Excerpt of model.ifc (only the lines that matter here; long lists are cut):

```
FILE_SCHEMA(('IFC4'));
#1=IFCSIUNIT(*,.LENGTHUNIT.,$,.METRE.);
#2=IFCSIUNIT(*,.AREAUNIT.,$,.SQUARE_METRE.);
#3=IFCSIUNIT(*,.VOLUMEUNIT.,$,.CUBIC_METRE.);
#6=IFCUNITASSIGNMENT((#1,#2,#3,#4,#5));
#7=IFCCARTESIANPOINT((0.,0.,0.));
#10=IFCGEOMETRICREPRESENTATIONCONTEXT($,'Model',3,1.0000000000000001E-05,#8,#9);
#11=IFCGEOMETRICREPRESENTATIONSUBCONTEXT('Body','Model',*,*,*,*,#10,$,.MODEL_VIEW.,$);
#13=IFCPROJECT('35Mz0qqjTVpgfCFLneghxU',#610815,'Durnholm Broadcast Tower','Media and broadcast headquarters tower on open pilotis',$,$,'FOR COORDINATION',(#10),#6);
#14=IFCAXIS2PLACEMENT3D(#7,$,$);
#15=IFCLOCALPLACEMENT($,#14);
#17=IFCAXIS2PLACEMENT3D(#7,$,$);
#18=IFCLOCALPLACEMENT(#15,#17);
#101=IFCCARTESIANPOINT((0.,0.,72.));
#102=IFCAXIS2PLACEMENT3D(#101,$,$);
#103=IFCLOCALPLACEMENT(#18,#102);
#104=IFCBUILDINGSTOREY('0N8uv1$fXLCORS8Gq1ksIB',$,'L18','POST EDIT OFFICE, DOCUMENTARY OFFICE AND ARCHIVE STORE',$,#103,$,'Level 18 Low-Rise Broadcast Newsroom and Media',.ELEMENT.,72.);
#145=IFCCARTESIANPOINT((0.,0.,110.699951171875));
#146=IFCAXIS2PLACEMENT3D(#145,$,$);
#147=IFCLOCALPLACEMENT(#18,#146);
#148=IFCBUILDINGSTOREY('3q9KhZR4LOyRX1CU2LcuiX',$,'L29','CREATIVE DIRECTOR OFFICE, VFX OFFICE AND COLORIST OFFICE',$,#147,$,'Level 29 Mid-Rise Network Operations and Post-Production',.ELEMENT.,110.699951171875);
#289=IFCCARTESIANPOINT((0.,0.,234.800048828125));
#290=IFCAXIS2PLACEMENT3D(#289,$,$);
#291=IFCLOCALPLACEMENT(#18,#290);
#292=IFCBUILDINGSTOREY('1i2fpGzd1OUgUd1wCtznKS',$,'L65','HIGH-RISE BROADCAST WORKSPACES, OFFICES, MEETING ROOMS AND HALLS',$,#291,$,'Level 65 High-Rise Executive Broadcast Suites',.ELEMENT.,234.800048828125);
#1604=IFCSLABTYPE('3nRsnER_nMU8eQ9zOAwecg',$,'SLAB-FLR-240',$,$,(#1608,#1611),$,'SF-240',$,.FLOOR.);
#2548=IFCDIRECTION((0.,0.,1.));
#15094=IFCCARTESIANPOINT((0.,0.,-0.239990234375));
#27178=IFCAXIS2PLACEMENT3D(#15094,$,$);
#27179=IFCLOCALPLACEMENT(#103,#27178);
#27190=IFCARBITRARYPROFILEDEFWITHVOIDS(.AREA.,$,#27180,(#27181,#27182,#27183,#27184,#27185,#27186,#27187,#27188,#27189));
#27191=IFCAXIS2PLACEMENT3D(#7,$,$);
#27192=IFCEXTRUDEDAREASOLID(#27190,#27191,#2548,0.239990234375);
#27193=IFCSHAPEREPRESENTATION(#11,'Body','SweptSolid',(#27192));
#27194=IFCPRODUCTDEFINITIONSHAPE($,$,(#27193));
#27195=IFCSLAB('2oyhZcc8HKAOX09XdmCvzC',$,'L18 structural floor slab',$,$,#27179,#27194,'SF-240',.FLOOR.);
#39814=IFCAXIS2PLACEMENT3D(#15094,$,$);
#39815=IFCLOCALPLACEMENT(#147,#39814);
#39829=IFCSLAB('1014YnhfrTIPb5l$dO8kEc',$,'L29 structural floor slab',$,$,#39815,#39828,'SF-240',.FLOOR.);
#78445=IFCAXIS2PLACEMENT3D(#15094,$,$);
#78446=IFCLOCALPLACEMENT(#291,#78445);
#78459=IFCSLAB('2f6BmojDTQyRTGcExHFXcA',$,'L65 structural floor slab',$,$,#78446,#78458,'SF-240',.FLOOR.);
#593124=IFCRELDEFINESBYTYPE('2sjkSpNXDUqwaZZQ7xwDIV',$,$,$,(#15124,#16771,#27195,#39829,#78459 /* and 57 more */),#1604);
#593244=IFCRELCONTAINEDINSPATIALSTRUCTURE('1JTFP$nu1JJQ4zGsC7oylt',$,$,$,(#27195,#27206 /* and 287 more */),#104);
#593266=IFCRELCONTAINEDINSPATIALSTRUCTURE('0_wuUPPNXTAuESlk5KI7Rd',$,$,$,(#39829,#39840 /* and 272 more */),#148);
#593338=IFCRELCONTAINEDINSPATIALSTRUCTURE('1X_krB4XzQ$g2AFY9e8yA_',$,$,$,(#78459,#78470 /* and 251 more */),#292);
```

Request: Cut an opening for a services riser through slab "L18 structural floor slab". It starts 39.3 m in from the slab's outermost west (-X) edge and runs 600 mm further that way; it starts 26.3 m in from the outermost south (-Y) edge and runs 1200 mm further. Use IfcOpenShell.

```python
import numpy as np
import ifcopenshell
import ifcopenshell.api.feature
import ifcopenshell.api.geometry
import ifcopenshell.api.root
import ifcopenshell.geom
import ifcopenshell.util.placement
import ifcopenshell.util.representation
import ifcopenshell.util.shape
import ifcopenshell.util.unit

model = ifcopenshell.open("model.ifc")
unit_scale = ifcopenshell.util.unit.calculate_unit_scale(model)
settings = ifcopenshell.geom.settings()


def volume(element):
    """Net volume in cubic metres, openings subtracted."""
    shape = ifcopenshell.geom.create_shape(settings, element)
    return ifcopenshell.util.shape.get_volume(shape.geometry)


slab = model.by_id(27195)
before = volume(slab)

# Extent in the slab's own axes, in metres. The edges named are its -X and -Y sides.
slab_shape = ifcopenshell.geom.create_shape(settings, slab)
vertices = ifcopenshell.util.shape.get_vertices(slab_shape.geometry)
x_min, y_min, bottom = vertices.min(axis=0)
top = vertices[:, 2].max()

opening = ifcopenshell.api.root.create_entity(model, ifc_class="IfcOpeningElement", name="Services riser opening", predefined_type="OPENING")
context = ifcopenshell.util.representation.get_context(model, "Model", "Body", "MODEL_VIEW")
width, depth = 0.6, 1.2
outline = [(0.0, 0.0), (width, 0.0), (width, depth), (0.0, depth), (0.0, 0.0)]
# Overshoot both faces by 50 mm so the cut is clean.
shape = ifcopenshell.api.geometry.add_slab_representation(
    model, context=context, depth=top - bottom + 0.1, polyline=outline
)
ifcopenshell.api.geometry.assign_representation(model, product=opening, representation=shape)

matrix = ifcopenshell.util.placement.get_local_placement(slab.ObjectPlacement)
matrix[:, 3] = matrix @ np.append(np.array([x_min + 39.3, y_min + 26.3, bottom - 0.05]) / unit_scale, 1.0)
ifcopenshell.api.geometry.edit_object_placement(model, product=opening, matrix=matrix, is_si=False)
ifcopenshell.api.feature.add_feature(model, feature=opening, element=slab)

after = volume(slab)

print(f"slab volume {before:.3f} -> {after:.3f} m3")

model.write("model_edited.ifc")
```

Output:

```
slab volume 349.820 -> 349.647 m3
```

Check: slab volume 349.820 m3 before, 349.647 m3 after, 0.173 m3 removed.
